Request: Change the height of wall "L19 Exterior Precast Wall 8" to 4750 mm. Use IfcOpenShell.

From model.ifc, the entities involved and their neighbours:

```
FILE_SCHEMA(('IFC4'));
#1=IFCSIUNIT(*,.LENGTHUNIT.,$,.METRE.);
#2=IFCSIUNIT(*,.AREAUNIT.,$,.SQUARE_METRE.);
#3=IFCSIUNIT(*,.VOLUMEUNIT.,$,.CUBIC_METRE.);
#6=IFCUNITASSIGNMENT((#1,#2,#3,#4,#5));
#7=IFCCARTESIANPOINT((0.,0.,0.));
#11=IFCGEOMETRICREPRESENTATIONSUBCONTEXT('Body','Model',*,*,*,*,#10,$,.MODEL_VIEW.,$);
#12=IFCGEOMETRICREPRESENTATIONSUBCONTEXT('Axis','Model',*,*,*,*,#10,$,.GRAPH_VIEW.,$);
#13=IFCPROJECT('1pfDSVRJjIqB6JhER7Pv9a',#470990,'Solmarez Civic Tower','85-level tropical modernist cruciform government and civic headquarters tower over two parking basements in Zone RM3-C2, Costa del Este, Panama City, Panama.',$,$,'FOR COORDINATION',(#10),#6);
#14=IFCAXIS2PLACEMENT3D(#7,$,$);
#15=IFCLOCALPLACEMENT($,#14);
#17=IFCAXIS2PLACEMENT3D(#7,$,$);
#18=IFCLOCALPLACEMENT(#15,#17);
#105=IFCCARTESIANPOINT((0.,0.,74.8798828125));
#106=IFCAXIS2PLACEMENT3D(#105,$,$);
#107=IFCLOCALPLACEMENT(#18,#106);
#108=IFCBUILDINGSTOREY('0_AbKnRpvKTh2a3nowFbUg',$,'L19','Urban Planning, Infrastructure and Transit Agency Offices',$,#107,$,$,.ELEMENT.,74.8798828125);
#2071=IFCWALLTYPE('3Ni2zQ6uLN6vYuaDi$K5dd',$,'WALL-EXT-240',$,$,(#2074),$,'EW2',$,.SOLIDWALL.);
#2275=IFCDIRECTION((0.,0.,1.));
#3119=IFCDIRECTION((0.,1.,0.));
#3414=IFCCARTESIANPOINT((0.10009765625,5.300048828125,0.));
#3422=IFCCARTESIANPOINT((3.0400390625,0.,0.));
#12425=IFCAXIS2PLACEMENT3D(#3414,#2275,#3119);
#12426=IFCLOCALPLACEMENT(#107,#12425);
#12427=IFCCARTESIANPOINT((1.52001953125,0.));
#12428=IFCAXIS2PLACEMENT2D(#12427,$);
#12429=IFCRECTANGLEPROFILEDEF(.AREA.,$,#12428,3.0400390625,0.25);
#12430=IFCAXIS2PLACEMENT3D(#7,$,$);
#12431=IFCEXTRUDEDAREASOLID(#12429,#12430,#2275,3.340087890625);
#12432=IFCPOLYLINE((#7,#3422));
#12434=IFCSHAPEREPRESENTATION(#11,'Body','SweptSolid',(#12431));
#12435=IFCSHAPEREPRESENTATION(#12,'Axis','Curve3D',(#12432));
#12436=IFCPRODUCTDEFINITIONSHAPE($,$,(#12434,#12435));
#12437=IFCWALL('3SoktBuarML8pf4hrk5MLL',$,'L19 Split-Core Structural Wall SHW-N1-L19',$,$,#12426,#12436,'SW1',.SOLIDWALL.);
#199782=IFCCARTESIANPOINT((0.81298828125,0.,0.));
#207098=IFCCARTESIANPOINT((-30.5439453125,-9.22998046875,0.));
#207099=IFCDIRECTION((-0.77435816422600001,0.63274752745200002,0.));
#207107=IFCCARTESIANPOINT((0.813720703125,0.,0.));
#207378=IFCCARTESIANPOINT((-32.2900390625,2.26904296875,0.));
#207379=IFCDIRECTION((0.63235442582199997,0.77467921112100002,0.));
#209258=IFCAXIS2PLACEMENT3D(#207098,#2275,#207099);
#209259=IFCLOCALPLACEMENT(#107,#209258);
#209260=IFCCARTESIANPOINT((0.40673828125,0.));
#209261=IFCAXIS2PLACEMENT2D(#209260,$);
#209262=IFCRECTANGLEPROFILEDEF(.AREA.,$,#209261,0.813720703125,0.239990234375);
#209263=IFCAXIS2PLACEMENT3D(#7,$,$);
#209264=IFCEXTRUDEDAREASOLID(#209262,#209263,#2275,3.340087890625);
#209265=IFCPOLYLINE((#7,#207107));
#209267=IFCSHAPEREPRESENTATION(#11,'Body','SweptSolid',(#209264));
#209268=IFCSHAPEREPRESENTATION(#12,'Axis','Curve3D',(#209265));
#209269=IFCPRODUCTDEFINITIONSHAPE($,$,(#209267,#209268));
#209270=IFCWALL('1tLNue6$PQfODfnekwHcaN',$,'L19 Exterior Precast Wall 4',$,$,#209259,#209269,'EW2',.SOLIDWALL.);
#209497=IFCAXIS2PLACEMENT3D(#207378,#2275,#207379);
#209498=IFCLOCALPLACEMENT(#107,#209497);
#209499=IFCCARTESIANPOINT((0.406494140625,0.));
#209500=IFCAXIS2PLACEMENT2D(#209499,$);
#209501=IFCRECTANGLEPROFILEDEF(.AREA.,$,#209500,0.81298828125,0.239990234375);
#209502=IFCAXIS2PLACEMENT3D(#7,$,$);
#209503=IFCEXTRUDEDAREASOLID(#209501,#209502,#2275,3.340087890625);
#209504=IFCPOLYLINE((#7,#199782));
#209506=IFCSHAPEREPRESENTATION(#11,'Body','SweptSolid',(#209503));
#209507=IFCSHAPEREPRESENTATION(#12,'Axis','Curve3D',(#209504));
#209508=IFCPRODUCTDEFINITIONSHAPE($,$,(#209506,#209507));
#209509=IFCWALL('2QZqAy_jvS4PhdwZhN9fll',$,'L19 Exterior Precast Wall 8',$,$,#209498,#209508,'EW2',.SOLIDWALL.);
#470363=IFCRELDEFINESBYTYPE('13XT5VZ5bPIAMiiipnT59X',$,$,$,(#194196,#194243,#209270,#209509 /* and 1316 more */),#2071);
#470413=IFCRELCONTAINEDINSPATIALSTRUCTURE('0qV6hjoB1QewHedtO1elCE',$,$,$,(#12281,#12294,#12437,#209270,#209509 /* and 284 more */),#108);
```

```python
import ifcopenshell
import ifcopenshell.geom
import ifcopenshell.util.representation
import ifcopenshell.util.shape

model = ifcopenshell.open("model.ifc")
settings = ifcopenshell.geom.settings()


def volume(element):
    """Net volume in cubic metres, openings subtracted."""
    shape = ifcopenshell.geom.create_shape(settings, element)
    return ifcopenshell.util.shape.get_volume(shape.geometry)


wall = model.by_guid("2QZqAy_jvS4PhdwZhN9fll")
before = volume(wall)

body = ifcopenshell.util.representation.get_representation(wall, "Model", "Body")
solid = body.Items[0]
old_height = solid.Depth
solid.Depth = 4.75
after = volume(wall)

print(f"height {old_height:g} -> {solid.Depth:g}, volume {before:.3f} -> {after:.3f} m3")

model.write("model_updated.ifc")
```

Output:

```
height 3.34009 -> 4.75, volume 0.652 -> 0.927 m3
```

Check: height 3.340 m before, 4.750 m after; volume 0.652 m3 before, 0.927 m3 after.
